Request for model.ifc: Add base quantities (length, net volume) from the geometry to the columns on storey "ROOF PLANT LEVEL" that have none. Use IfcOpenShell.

First a look at what the model holds.

```python
import ifcopenshell
import ifcopenshell.util.element
import ifcopenshell.util.unit

model = ifcopenshell.open("model.ifc")
print(model.schema)
for unit_type in ("LENGTHUNIT", "AREAUNIT", "VOLUMEUNIT"):
    print(unit_type, ifcopenshell.util.unit.calculate_unit_scale(model, unit_type))
storey = next(s for s in model.by_type("IfcBuildingStorey") if s.Name == "ROOF PLANT LEVEL")
columns = [e for e in ifcopenshell.util.element.get_decomposition(storey) if e.is_a("IfcColumn")]
for e in sorted(columns, key=lambda e: e.id()):
    print(e.id(), e.is_a(), e.Name, list(ifcopenshell.util.element.get_psets(e, qtos_only=True)), sep=" | ")
```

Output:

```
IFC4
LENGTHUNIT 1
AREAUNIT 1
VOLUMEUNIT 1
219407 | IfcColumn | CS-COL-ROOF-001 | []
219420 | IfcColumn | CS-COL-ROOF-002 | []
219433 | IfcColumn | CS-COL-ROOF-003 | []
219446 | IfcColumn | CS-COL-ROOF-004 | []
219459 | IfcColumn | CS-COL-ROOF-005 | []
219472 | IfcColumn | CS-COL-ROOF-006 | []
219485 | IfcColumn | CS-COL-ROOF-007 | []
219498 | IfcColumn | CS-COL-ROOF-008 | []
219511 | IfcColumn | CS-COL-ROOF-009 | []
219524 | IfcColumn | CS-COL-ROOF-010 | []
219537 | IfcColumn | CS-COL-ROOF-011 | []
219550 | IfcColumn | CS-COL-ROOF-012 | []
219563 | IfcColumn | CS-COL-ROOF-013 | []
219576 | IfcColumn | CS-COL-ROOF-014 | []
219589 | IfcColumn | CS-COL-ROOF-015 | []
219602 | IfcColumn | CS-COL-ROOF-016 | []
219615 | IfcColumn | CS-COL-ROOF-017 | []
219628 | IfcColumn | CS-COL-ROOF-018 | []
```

```python
import ifcopenshell
import ifcopenshell.api.pset
import ifcopenshell.geom
import ifcopenshell.util.element
import ifcopenshell.util.shape
import ifcopenshell.util.unit

model = ifcopenshell.open("model.ifc")
unit_scale = ifcopenshell.util.unit.calculate_unit_scale(model)
volume_scale = ifcopenshell.util.unit.calculate_unit_scale(model, "VOLUMEUNIT")
settings = ifcopenshell.geom.settings()

storey = next(s for s in model.by_type("IfcBuildingStorey") if s.Name == "ROOF PLANT LEVEL")
columns = [e for e in ifcopenshell.util.element.get_decomposition(storey) if e.is_a("IfcColumn")]

for e in sorted(columns, key=lambda e: e.id()):
    if ifcopenshell.util.element.get_psets(e, qtos_only=True, should_inherit=False):
        continue
    # Geometry comes back in metres, in the element's own axes.
    shape = ifcopenshell.geom.create_shape(settings, e)
    values = {
        "Length": ifcopenshell.util.shape.get_z(shape.geometry) / unit_scale,
        "NetVolume": ifcopenshell.util.shape.get_volume(shape.geometry) / volume_scale,
    }
    qto = ifcopenshell.api.pset.add_qto(model, product=e, name="Qto_ColumnBaseQuantities")
    ifcopenshell.api.pset.edit_qto(model, qto=qto, properties=values)
    print(e.id(), {k: round(v, 3) for k, v in values.items()})

model.write("model_v2.ifc")
```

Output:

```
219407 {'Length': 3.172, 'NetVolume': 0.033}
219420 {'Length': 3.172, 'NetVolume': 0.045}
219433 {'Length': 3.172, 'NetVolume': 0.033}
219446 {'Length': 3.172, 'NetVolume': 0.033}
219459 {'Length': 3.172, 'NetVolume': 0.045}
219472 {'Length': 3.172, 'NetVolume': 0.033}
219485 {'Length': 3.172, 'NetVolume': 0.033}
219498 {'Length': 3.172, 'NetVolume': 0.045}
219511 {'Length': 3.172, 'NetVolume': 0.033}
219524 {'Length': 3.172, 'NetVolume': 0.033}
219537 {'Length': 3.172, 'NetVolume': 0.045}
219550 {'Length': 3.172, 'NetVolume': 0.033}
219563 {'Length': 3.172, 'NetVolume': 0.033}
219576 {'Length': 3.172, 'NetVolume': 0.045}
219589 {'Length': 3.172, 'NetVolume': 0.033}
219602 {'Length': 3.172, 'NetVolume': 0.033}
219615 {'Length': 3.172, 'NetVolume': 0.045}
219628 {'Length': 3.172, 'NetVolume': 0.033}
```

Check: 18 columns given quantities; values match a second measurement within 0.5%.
